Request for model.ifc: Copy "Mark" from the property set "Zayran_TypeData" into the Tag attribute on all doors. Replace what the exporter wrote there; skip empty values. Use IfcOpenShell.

First a look at what the model holds.

```python
import ifcopenshell
import ifcopenshell.util.element

model = ifcopenshell.open("model.ifc")
print(model.schema)
doors = model.by_type("IfcDoor")
print(len(doors), "doors")
for e in doors[:8]:
    source = ifcopenshell.util.element.get_pset(e, "Zayran_TypeData", "Mark")
    target = e.Tag
    print(e.id(), repr(source), repr(target), sep=" | ")
```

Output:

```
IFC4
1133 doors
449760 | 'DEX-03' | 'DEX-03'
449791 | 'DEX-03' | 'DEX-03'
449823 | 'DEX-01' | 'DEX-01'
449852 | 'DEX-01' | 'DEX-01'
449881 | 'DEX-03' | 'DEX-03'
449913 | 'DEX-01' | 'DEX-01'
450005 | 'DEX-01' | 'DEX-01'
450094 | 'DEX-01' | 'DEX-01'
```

```python
import ifcopenshell
import ifcopenshell.util.element

model = ifcopenshell.open("model.ifc")

count = 0
for e in model.by_type("IfcDoor"):
    value = ifcopenshell.util.element.get_pset(e, "Zayran_TypeData", "Mark")
    current = e.Tag
    if not value or not value.strip() or current == value:
        continue
    e.Tag = value
    count += 1

print(count, "doors updated")

model.write("model_v2.ifc")
```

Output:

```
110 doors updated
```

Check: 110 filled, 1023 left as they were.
